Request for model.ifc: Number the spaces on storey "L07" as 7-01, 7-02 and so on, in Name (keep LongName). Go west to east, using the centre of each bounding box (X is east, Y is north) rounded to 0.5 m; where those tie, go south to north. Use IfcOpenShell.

First a look at what the model holds.

```python
import ifcopenshell
import ifcopenshell.util.element
import ifcopenshell.util.placement

model = ifcopenshell.open("model.ifc")
print(model.schema)
storey = next(s for s in model.by_type("IfcBuildingStorey") if s.Name == "L07")
spaces = [e for e in ifcopenshell.util.element.get_decomposition(storey) if e.is_a("IfcSpace")]
for e in sorted(spaces, key=lambda e: e.id()):
    origin = ifcopenshell.util.placement.get_local_placement(e.ObjectPlacement)[:3, 3]
    print(e.id(), e.Name, e.LongName, origin.round(2) + 0.0, sep=" | ")
```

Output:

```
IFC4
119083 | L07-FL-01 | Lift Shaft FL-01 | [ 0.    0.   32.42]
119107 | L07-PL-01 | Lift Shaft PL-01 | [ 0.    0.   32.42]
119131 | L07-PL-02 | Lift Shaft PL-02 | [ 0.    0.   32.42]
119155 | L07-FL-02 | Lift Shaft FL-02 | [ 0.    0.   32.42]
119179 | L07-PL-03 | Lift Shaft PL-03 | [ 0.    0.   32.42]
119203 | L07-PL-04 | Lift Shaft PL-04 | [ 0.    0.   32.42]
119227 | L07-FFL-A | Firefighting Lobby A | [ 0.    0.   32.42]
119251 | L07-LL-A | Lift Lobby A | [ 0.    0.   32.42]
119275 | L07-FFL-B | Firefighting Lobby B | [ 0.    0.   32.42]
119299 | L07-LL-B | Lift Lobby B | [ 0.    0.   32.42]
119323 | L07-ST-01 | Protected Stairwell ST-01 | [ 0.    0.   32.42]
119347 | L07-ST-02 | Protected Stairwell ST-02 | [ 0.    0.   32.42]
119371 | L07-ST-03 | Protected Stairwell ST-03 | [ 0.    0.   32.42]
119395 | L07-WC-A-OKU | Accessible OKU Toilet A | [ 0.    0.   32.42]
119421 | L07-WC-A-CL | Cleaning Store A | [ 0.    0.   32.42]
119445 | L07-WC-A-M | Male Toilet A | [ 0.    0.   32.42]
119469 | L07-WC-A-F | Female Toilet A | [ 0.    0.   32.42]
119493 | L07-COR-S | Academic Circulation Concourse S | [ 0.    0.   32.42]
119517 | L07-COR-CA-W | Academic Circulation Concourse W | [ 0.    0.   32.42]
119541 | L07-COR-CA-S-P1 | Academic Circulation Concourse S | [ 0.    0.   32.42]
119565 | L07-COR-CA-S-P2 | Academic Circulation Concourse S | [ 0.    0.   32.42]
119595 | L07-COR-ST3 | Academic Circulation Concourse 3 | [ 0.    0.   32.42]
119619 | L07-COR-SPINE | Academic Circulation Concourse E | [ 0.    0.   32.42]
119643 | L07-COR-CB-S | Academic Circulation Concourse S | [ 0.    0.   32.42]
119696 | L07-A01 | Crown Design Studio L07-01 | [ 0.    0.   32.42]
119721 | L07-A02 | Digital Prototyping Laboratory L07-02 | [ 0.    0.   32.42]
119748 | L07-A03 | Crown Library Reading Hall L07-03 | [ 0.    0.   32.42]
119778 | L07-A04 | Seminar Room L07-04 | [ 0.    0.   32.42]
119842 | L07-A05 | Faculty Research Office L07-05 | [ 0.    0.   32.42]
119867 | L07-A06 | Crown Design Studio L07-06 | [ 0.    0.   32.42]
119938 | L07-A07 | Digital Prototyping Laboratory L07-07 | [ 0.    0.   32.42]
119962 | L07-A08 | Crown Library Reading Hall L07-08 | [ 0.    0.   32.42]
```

```python
import ifcopenshell
import ifcopenshell.geom
import ifcopenshell.util.element
import ifcopenshell.util.shape

model = ifcopenshell.open("model.ifc")
settings = ifcopenshell.geom.settings()
settings.set("use-world-coords", True)


def centre(element):
    shape = ifcopenshell.geom.create_shape(settings, element)
    return ifcopenshell.util.shape.get_bbox_centroid(shape.geometry)


storey = next(s for s in model.by_type("IfcBuildingStorey") if s.Name == "L07")
spaces = [e for e in ifcopenshell.util.element.get_decomposition(storey) if e.is_a("IfcSpace")]

# Insertion points can sit at a corner or the storey origin, so sort by the geometry (in metres).
centres = {e: centre(e) for e in spaces}
spaces.sort(key=lambda e: (round(centres[e][0] / 0.5), centres[e][1]))

for i, e in enumerate(spaces, start=1):
    number = f"7-{i:02d}"
    e.Name = number
    print(e.id(), number)

model.write("model_edited.ifc")
```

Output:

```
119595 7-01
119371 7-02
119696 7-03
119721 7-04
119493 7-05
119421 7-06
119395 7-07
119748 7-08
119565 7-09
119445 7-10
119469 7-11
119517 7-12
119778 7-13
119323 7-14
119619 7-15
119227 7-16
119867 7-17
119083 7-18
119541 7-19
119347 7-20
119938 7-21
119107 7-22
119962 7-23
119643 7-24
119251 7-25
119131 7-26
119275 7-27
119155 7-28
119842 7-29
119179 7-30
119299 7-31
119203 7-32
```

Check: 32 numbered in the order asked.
